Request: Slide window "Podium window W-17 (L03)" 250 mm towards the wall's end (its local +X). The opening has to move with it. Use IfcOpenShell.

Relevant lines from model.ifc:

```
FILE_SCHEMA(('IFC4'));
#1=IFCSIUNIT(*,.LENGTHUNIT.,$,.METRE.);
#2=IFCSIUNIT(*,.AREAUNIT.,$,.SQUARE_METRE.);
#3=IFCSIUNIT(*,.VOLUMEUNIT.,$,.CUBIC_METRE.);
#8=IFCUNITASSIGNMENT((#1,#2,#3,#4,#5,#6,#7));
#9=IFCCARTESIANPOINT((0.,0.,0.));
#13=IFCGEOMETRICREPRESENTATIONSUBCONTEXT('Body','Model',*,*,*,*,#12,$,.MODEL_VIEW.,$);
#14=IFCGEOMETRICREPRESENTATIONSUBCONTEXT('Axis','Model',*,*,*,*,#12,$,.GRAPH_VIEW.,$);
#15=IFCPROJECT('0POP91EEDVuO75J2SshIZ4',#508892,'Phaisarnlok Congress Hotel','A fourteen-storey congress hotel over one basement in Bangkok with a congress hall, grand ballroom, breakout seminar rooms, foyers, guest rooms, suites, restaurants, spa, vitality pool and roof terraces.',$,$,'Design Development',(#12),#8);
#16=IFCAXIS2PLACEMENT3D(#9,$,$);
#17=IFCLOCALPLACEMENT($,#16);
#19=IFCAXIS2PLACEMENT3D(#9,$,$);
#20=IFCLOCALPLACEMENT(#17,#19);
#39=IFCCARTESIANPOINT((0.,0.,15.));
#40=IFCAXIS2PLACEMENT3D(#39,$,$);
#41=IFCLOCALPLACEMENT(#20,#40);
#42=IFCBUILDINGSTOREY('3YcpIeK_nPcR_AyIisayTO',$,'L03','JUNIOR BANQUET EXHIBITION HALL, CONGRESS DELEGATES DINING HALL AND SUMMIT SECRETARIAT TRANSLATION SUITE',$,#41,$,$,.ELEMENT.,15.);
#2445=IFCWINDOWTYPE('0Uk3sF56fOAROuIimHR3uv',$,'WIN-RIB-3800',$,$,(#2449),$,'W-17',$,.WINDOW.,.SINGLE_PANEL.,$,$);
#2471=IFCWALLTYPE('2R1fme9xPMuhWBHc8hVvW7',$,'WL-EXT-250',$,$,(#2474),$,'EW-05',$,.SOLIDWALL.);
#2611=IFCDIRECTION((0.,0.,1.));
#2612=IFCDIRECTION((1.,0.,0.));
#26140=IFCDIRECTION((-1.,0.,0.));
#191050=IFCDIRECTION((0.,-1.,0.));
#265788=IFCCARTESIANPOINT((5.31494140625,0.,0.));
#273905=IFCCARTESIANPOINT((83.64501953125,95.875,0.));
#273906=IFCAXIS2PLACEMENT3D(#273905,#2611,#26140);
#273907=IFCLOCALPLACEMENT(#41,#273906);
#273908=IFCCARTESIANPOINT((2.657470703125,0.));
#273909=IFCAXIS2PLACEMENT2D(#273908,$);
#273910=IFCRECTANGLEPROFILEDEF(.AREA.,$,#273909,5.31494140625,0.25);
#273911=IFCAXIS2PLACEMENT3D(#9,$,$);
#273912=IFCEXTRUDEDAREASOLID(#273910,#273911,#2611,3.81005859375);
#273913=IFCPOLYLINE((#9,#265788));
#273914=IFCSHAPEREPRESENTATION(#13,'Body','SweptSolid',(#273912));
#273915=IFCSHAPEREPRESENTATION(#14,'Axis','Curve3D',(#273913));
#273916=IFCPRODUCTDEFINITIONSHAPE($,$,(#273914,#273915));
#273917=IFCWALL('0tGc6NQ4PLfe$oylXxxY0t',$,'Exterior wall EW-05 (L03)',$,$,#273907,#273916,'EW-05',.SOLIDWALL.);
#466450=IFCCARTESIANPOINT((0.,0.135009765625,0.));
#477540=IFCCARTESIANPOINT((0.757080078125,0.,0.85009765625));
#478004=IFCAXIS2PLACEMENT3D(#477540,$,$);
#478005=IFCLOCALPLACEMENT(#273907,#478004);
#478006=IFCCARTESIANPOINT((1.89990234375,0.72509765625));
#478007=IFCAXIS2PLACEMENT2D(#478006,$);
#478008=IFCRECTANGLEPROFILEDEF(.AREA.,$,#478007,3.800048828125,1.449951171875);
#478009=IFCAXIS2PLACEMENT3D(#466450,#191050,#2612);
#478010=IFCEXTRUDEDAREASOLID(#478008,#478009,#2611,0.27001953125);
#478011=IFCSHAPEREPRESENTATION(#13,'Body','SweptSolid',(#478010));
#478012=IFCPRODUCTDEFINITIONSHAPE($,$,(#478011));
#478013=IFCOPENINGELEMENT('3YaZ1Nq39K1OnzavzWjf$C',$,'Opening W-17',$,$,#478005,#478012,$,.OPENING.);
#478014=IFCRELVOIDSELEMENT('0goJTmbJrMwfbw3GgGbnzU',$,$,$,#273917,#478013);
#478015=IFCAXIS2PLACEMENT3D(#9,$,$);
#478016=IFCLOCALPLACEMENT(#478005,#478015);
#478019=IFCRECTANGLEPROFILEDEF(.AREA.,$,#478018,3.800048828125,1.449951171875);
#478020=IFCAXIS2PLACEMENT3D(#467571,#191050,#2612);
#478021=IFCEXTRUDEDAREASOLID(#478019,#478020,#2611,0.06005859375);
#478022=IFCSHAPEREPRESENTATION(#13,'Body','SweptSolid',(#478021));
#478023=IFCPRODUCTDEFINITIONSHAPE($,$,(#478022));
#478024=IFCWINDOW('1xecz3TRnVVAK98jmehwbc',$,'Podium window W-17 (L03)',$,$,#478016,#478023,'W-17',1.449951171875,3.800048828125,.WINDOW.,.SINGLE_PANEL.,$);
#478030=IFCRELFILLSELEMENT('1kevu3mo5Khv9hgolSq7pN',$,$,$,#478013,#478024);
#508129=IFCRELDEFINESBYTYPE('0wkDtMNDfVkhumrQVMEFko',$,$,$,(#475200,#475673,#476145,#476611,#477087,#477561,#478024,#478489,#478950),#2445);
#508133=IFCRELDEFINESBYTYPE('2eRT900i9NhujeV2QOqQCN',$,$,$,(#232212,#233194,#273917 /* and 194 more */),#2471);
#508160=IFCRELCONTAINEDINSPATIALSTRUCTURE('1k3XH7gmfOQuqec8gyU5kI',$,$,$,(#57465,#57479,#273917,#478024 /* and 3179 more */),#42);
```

```python
import ifcopenshell
import ifcopenshell.api.geometry
import ifcopenshell.util.placement
import ifcopenshell.util.unit

model = ifcopenshell.open("model.ifc")
unit_scale = ifcopenshell.util.unit.calculate_unit_scale(model)

window = model.by_id(478024)
opening = window.FillsVoids[0].RelatingOpeningElement
wall = opening.VoidsElements[0].RelatingBuildingElement

wall_matrix = ifcopenshell.util.placement.get_local_placement(wall.ObjectPlacement)
shift = wall_matrix[:3, 0] * 0.25 / unit_scale
before = ifcopenshell.util.placement.get_local_placement(window.ObjectPlacement)[:3, 3].copy()

# The window is placed relative to its opening, so it follows when the opening moves.
matrix = ifcopenshell.util.placement.get_local_placement(opening.ObjectPlacement)
matrix[:3, 3] += shift
ifcopenshell.api.geometry.edit_object_placement(
    model, product=opening, matrix=matrix, is_si=False, should_transform_children=True
)

after = ifcopenshell.util.placement.get_local_placement(window.ObjectPlacement)[:3, 3]
print("window moved by", (after - before).round(3) + 0.0)

model.write("model_edited.ifc")
```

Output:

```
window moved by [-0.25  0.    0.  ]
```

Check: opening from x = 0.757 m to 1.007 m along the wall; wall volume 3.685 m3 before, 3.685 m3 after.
